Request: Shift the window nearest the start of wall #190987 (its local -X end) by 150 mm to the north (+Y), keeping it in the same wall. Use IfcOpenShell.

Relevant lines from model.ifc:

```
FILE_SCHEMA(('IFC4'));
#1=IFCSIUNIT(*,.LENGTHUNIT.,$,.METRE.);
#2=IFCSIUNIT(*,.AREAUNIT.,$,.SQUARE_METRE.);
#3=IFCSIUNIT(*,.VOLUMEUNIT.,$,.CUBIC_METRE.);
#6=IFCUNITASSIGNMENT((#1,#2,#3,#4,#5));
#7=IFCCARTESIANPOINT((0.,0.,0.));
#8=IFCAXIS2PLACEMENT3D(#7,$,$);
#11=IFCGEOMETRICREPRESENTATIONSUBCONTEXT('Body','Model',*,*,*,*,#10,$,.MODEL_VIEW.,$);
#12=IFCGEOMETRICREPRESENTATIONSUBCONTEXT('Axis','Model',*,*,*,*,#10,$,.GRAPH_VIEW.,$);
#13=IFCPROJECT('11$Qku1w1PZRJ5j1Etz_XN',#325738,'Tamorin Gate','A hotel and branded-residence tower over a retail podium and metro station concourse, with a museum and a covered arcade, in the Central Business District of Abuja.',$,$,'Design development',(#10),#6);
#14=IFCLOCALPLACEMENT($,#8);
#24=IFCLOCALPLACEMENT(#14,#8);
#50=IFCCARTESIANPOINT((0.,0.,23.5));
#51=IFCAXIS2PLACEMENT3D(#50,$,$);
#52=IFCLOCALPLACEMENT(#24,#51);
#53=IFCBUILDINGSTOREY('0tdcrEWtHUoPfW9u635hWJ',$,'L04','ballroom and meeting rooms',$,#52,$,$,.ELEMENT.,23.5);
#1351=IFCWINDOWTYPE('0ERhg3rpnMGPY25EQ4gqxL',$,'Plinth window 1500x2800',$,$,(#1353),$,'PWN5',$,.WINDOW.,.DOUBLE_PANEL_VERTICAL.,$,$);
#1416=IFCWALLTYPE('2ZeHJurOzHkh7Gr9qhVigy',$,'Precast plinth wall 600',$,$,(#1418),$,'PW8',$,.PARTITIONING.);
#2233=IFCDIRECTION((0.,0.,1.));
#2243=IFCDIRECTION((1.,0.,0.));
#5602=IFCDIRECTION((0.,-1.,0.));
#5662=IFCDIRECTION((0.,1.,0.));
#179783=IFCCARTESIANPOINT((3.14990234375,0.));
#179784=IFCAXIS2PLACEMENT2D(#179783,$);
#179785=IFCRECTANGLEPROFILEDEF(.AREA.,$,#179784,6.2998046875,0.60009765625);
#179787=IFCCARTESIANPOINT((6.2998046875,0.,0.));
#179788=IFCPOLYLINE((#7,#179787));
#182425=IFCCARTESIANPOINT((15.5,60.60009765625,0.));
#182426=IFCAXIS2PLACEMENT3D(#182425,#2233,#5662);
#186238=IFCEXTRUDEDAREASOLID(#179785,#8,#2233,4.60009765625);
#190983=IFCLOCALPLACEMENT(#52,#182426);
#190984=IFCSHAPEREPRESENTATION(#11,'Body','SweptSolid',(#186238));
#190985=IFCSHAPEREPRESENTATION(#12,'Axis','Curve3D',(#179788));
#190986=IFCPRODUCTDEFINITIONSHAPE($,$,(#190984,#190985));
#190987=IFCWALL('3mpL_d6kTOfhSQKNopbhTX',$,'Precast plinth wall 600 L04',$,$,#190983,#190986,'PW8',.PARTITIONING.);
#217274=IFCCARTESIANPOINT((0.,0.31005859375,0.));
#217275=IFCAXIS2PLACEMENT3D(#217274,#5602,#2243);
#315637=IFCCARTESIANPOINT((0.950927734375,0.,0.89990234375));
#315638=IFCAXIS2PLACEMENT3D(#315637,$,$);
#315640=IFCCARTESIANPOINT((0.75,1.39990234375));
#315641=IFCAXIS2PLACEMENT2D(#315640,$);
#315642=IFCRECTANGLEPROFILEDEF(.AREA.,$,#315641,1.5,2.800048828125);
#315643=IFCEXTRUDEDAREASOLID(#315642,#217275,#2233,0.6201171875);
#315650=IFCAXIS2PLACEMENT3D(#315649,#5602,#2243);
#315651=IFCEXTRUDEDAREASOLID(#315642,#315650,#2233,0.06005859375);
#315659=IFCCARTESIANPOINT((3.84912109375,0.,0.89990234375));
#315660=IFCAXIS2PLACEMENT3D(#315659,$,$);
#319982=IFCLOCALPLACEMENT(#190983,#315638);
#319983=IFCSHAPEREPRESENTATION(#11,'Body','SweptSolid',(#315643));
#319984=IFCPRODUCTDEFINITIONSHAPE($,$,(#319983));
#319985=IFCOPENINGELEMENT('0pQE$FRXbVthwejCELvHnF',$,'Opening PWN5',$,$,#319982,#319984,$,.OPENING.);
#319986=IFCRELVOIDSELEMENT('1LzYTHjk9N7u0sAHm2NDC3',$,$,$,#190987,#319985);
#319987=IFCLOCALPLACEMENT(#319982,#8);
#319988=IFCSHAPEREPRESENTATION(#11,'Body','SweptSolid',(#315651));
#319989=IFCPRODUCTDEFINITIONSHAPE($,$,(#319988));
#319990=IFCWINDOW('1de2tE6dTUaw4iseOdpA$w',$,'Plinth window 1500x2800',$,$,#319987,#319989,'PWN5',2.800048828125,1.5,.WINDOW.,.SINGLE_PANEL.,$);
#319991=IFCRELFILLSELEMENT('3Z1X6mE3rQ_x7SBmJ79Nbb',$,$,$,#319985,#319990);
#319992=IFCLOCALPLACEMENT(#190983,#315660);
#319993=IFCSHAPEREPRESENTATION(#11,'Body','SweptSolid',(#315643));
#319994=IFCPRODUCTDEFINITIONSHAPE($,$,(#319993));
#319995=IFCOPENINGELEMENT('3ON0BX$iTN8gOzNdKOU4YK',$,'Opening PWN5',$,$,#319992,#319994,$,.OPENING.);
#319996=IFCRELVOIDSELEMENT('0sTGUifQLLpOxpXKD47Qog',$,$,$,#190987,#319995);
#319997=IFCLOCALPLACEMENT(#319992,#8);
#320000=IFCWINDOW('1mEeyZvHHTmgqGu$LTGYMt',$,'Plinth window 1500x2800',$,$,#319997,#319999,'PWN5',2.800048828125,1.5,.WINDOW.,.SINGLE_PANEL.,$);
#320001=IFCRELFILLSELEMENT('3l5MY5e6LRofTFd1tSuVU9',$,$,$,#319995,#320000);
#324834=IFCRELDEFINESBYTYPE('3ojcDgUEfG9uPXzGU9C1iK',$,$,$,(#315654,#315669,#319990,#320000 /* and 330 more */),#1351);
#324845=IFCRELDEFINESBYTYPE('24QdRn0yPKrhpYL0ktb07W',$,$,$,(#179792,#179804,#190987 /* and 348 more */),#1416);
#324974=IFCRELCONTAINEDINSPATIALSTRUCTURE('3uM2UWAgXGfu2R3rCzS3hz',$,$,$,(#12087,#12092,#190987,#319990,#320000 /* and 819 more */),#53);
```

```python
import ifcopenshell
import ifcopenshell.api.geometry
import ifcopenshell.util.placement
import ifcopenshell.util.unit

model = ifcopenshell.open("model.ifc")
unit_scale = ifcopenshell.util.unit.calculate_unit_scale(model)

window = model.by_guid("1de2tE6dTUaw4iseOdpA$w")
opening = window.FillsVoids[0].RelatingOpeningElement
wall = opening.VoidsElements[0].RelatingBuildingElement

wall_matrix = ifcopenshell.util.placement.get_local_placement(wall.ObjectPlacement)
shift = wall_matrix[:3, 0] * 0.15 / unit_scale
before = ifcopenshell.util.placement.get_local_placement(window.ObjectPlacement)[:3, 3].copy()

# The window is placed relative to its opening, so it follows when the opening moves.
matrix = ifcopenshell.util.placement.get_local_placement(opening.ObjectPlacement)
matrix[:3, 3] += shift
ifcopenshell.api.geometry.edit_object_placement(
    model, product=opening, matrix=matrix, is_si=False, should_transform_children=True
)

after = ifcopenshell.util.placement.get_local_placement(window.ObjectPlacement)[:3, 3]
print("window moved by", (after - before).round(3) + 0.0)

model.write("model_v2.ifc")
```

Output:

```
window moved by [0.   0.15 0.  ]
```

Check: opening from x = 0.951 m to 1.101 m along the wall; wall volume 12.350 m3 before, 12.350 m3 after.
